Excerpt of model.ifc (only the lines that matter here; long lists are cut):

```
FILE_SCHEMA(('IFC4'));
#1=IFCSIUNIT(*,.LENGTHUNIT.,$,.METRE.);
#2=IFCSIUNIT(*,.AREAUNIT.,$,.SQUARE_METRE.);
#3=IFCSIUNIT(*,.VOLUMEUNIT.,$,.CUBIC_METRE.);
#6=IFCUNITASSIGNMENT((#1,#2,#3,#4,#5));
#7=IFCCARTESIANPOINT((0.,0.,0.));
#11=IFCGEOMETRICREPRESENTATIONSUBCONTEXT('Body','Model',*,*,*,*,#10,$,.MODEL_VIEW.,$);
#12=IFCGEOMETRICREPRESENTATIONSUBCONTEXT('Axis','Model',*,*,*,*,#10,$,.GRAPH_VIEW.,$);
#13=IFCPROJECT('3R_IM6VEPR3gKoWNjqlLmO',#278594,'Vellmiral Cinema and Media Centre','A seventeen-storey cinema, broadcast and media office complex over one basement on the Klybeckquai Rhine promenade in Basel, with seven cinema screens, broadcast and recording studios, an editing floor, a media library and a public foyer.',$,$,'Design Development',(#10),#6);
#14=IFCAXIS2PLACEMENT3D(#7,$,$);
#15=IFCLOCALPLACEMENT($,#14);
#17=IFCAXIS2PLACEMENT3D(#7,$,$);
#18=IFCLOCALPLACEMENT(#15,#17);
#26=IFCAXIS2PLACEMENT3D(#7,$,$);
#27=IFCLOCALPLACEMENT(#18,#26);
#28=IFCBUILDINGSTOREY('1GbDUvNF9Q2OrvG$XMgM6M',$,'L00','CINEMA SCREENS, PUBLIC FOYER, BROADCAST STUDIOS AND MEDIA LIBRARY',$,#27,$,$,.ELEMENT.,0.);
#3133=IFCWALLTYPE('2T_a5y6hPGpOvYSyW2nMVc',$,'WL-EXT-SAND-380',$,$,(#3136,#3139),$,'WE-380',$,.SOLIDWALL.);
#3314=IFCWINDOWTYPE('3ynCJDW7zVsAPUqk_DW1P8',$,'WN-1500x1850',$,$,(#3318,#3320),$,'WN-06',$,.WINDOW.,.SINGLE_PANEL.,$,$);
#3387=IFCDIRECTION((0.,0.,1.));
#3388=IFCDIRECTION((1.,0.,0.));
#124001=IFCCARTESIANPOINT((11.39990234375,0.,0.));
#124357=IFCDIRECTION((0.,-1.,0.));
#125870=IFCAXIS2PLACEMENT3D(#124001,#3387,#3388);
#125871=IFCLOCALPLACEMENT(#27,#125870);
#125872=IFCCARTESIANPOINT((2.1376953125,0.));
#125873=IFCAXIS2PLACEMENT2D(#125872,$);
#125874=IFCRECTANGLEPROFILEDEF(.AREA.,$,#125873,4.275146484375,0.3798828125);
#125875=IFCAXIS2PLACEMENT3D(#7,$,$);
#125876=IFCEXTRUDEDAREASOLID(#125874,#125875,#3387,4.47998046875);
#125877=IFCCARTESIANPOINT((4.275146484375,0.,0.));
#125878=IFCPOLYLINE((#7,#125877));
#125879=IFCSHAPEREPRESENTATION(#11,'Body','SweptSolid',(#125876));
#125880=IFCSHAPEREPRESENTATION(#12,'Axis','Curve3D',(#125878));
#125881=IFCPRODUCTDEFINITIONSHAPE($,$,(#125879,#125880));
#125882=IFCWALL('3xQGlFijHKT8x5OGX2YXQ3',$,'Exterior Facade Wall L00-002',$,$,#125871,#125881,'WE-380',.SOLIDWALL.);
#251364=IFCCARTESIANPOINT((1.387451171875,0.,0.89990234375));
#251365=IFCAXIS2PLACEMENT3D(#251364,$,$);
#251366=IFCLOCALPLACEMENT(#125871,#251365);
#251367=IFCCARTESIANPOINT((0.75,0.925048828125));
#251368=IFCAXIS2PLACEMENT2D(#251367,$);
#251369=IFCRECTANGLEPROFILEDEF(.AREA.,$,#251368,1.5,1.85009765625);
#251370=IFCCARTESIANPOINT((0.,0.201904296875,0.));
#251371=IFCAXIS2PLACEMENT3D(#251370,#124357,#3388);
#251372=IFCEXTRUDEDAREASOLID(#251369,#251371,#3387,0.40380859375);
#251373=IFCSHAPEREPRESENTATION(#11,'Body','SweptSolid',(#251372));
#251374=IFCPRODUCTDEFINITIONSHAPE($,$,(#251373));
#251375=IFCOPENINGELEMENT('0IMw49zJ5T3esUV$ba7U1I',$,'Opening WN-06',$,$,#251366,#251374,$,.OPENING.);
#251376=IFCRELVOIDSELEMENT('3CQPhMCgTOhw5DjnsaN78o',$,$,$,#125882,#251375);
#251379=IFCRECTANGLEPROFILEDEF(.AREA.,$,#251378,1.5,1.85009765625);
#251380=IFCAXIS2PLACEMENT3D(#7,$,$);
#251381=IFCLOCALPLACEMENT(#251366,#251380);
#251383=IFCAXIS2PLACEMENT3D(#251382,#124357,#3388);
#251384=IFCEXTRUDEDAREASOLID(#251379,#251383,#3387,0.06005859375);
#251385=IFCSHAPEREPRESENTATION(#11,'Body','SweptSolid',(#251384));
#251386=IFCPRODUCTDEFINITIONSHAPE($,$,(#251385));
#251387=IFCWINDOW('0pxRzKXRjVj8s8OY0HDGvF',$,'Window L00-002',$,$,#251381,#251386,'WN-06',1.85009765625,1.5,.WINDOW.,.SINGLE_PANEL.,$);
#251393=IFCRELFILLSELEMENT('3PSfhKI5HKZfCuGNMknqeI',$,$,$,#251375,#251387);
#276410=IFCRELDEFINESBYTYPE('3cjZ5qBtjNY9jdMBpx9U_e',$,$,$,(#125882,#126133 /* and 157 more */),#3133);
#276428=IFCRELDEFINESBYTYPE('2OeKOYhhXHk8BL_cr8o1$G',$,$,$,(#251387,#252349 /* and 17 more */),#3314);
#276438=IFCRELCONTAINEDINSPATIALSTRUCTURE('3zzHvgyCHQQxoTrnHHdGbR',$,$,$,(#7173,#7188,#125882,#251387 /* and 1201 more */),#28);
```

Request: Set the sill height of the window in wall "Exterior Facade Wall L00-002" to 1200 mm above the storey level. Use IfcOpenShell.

```python
import numpy as np
import ifcopenshell
import ifcopenshell.api.geometry
import ifcopenshell.geom
import ifcopenshell.util.element
import ifcopenshell.util.placement
import ifcopenshell.util.shape
import ifcopenshell.util.unit

model = ifcopenshell.open("model.ifc")
unit_scale = ifcopenshell.util.unit.calculate_unit_scale(model)

window = model.by_guid("0pxRzKXRjVj8s8OY0HDGvF")
opening = window.FillsVoids[0].RelatingOpeningElement
storey = ifcopenshell.util.element.get_container(window, ifc_class="IfcBuildingStorey")
level = ifcopenshell.util.placement.get_local_placement(storey.ObjectPlacement)[2, 3]

# The opening's origin need not be at the sill, so measure its lowest point.
shape = ifcopenshell.geom.create_shape(ifcopenshell.geom.settings(), opening)
bottom = ifcopenshell.util.shape.get_shape_bottom_elevation(shape, shape.geometry) / unit_scale
dz = level + 1.2 / unit_scale - bottom

shift = np.array([0.0, 0.0, dz])
# The window is placed relative to its opening, so it follows when the opening moves.
matrix = ifcopenshell.util.placement.get_local_placement(opening.ObjectPlacement)
matrix[:3, 3] += shift
ifcopenshell.api.geometry.edit_object_placement(
    model, product=opening, matrix=matrix, is_si=False, should_transform_children=True
)

print(f"moved by {dz * unit_scale:+.3f} m")

model.write("model_rev.ifc")
```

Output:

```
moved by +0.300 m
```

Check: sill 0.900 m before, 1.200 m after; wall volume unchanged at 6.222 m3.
